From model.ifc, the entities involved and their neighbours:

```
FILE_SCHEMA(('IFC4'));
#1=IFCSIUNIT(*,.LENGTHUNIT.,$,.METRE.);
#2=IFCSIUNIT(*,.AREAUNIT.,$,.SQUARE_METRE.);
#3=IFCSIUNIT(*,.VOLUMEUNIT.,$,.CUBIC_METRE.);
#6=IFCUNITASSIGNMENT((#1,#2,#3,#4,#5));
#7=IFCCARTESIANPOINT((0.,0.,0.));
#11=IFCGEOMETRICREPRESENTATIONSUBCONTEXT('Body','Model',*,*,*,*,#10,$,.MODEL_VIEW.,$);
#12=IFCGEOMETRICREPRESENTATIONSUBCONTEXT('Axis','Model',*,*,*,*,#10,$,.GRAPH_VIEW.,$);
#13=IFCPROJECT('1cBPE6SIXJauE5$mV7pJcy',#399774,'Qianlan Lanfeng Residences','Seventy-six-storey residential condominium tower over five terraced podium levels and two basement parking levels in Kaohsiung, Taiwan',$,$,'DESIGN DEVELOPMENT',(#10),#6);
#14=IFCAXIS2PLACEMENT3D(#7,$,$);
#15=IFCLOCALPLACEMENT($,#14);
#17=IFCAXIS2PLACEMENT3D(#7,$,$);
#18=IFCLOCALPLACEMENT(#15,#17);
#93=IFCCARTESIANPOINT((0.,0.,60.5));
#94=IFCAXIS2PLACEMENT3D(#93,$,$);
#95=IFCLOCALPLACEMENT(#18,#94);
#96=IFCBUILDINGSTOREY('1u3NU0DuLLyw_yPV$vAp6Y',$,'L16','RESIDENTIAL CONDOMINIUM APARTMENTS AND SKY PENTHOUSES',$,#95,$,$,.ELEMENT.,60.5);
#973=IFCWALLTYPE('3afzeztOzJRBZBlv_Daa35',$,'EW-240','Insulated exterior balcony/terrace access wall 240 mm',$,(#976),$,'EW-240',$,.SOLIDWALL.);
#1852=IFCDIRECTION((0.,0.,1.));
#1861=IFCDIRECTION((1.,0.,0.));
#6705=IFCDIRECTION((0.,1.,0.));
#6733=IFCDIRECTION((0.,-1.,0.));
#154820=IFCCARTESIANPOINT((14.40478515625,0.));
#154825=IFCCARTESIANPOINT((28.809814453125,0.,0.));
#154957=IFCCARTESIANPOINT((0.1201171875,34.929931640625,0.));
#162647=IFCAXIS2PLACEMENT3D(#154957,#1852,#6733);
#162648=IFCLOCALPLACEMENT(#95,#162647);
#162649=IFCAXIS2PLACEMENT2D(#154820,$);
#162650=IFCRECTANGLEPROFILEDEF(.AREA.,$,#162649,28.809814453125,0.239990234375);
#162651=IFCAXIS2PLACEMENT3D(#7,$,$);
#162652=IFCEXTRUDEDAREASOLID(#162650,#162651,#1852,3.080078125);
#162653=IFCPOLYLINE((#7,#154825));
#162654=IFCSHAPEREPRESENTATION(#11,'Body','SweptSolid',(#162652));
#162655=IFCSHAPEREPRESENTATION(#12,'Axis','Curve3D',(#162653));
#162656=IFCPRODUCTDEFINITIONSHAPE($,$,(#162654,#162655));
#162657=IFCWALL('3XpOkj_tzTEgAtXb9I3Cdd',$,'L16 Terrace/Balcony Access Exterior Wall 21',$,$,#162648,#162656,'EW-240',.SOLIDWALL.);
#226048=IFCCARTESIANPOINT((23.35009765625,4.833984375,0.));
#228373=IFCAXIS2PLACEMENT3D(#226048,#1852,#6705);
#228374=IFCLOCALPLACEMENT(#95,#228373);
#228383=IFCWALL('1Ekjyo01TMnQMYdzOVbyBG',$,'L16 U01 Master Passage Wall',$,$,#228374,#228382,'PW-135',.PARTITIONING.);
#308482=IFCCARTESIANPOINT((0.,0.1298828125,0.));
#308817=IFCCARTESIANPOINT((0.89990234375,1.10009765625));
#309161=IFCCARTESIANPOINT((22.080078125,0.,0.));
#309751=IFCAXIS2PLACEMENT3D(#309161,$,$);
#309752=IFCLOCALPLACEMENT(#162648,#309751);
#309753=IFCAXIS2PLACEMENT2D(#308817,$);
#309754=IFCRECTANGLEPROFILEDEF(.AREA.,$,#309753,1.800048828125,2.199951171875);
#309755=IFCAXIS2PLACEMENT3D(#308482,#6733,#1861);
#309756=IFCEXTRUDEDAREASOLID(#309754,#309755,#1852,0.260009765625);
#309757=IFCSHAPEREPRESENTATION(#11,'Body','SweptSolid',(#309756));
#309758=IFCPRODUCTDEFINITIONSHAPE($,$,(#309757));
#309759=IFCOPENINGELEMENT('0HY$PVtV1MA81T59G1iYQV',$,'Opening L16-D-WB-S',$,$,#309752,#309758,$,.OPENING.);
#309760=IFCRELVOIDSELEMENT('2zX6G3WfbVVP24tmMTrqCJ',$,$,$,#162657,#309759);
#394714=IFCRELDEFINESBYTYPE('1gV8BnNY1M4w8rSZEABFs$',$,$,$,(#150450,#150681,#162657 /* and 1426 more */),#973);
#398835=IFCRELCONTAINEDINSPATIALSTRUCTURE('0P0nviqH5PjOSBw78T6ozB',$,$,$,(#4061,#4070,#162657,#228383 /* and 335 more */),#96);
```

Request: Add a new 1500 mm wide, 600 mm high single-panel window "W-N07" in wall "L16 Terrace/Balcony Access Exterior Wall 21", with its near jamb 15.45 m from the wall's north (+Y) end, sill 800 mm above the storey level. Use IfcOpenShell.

```python
import numpy as np
import ifcopenshell
import ifcopenshell.api.feature
import ifcopenshell.api.geometry
import ifcopenshell.api.root
import ifcopenshell.api.spatial
import ifcopenshell.geom
import ifcopenshell.util.element
import ifcopenshell.util.placement
import ifcopenshell.util.representation
import ifcopenshell.util.shape
import ifcopenshell.util.unit

model = ifcopenshell.open("model.ifc")
unit_scale = ifcopenshell.util.unit.calculate_unit_scale(model)
settings = ifcopenshell.geom.settings()


def volume(element):
    """Net volume in cubic metres, openings subtracted."""
    shape = ifcopenshell.geom.create_shape(settings, element)
    return ifcopenshell.util.shape.get_volume(shape.geometry)


wall = model.by_guid("3XpOkj_tzTEgAtXb9I3Cdd")
storey = ifcopenshell.util.element.get_container(wall, ifc_class="IfcBuildingStorey")
context = ifcopenshell.util.representation.get_context(model, "Model", "Body", "MODEL_VIEW")
before = volume(wall)

width, height, from_end, sill = 1.5, 0.6, 15.45, 0.8  # metres

# The wall runs along its own X axis, and the end named is its -X end.
wall_shape = ifcopenshell.geom.create_shape(settings, wall)
x, y, z = ifcopenshell.util.shape.get_vertices(wall_shape.geometry).T
start = x.min() + from_end
face, thickness = float(y.min()), float(y.max() - y.min())
wall_matrix = ifcopenshell.util.placement.get_local_placement(wall.ObjectPlacement)
level = ifcopenshell.util.placement.get_local_placement(storey.ObjectPlacement)[2, 3]


def in_wall(x, y):
    """Placement at x, y metres in the wall's axes, at sill height."""
    matrix = wall_matrix.copy()
    matrix[:, 3] = wall_matrix @ np.array([x / unit_scale, y / unit_scale, 0.0, 1.0])
    matrix[2, 3] = level + sill / unit_scale
    return matrix


# Opening: a box that overshoots both wall faces by 50 mm.
opening = ifcopenshell.api.root.create_entity(model, ifc_class="IfcOpeningElement", predefined_type="OPENING")
box = ifcopenshell.api.geometry.add_wall_representation(
    model, context=context, length=width, height=height, thickness=thickness + 0.1
)
ifcopenshell.api.geometry.assign_representation(model, product=opening, representation=box)
ifcopenshell.api.geometry.edit_object_placement(model, product=opening, matrix=in_wall(start, face - 0.05), is_si=False)
ifcopenshell.api.feature.add_feature(model, feature=opening, element=wall)

window = ifcopenshell.api.root.create_entity(model, ifc_class="IfcWindow", name="W-N07", predefined_type="WINDOW")
window.OverallWidth, window.OverallHeight = width / unit_scale, height / unit_scale
window.PartitioningType = "SINGLE_PANEL"
body = ifcopenshell.api.geometry.add_window_representation(
    model,
    context=context,
    overall_width=window.OverallWidth,
    overall_height=window.OverallHeight,
    partition_type="SINGLE_PANEL",
)
ifcopenshell.api.geometry.assign_representation(model, product=window, representation=body)
ifcopenshell.api.spatial.assign_container(model, products=[window], relating_structure=storey)
ifcopenshell.api.feature.add_filling(model, opening=opening, element=window)

# Centre the window in the wall's thickness.
ifcopenshell.api.geometry.edit_object_placement(model, product=window, matrix=in_wall(start, face), is_si=False)
window_shape = ifcopenshell.geom.create_shape(settings, window)
depth = ifcopenshell.util.shape.get_vertices(window_shape.geometry)[:, 1]
offset = face + thickness / 2 - (depth.min() + depth.max()) / 2
ifcopenshell.api.geometry.edit_object_placement(model, product=window, matrix=in_wall(start, offset), is_si=False)

after = volume(wall)

print(f"wall volume {before:.3f} -> {after:.3f} m3")

model.write("model_v2.ifc")
```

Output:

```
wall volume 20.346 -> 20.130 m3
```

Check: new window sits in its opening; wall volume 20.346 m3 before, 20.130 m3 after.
